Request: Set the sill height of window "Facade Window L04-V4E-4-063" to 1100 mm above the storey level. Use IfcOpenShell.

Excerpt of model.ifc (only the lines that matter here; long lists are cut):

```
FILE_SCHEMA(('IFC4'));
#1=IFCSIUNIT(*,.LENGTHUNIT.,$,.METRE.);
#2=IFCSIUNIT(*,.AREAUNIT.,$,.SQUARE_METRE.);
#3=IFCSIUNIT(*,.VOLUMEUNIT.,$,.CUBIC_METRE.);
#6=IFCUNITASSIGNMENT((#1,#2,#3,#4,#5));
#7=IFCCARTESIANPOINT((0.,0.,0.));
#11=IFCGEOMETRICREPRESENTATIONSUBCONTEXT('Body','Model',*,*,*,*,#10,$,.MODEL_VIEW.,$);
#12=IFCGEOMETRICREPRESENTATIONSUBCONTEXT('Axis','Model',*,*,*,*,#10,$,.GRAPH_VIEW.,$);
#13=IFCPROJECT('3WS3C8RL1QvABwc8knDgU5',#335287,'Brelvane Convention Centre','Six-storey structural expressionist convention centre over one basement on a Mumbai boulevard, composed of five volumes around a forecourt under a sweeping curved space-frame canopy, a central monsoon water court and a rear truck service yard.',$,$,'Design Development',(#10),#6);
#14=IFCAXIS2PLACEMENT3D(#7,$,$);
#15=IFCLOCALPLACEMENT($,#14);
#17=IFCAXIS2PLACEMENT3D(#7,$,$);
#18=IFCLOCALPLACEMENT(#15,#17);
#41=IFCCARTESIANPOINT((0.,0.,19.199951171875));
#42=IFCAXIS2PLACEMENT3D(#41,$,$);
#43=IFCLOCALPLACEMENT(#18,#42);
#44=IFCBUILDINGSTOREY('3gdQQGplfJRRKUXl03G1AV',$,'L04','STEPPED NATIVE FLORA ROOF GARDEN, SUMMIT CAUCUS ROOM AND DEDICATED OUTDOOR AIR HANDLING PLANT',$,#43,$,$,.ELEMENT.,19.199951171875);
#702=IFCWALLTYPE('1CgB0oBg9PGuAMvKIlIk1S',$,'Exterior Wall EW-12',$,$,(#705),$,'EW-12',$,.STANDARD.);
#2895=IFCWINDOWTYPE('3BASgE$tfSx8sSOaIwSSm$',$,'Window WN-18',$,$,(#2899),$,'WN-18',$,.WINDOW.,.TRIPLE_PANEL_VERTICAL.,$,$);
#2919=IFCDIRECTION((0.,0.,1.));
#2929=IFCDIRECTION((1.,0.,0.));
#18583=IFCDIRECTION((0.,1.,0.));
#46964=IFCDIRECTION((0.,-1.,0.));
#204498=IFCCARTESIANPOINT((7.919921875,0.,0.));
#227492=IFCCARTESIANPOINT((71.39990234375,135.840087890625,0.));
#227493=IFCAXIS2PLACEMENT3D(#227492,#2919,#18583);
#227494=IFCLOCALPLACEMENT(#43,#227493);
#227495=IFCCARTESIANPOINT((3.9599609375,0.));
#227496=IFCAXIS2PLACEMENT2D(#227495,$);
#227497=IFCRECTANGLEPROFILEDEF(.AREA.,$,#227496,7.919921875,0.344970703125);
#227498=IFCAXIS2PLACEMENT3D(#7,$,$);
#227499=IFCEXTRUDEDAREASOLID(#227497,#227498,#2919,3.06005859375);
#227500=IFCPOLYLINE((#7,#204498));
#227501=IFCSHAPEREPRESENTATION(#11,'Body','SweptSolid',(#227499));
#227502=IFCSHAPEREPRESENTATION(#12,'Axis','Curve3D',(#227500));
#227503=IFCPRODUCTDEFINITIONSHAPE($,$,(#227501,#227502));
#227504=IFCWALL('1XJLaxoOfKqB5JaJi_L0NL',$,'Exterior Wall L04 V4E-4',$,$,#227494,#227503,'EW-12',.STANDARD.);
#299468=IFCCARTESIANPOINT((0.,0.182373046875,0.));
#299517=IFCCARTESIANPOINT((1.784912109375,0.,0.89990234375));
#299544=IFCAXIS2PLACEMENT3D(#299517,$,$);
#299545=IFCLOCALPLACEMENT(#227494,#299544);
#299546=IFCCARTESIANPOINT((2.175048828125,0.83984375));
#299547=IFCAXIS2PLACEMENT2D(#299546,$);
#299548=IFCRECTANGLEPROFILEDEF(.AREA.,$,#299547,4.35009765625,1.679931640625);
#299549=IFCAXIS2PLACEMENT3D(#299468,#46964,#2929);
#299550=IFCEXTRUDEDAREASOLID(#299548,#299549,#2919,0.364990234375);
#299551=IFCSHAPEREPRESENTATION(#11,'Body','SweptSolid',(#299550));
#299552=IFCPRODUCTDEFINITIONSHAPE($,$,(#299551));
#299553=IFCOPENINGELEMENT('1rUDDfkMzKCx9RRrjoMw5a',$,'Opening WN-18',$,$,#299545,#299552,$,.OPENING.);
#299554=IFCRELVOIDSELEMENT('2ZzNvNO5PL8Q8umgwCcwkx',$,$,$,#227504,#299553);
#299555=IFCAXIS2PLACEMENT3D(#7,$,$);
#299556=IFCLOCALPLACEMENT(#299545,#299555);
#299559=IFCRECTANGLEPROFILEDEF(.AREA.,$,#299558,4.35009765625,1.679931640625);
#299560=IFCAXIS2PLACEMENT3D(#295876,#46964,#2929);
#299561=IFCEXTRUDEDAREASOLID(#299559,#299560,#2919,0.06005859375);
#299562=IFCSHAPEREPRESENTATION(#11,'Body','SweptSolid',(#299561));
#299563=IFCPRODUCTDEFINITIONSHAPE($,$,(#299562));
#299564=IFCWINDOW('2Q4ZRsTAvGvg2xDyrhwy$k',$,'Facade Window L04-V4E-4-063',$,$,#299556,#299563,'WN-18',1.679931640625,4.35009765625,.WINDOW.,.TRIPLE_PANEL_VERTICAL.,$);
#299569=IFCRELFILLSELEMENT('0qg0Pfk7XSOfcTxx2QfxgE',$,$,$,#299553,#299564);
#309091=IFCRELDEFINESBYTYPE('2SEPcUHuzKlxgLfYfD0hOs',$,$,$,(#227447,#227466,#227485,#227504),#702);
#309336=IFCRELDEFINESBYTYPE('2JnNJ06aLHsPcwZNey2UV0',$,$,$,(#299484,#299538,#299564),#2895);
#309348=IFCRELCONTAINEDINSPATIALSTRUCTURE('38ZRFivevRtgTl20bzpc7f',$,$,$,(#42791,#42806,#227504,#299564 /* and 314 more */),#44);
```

```python
import numpy as np
import ifcopenshell
import ifcopenshell.api.geometry
import ifcopenshell.geom
import ifcopenshell.util.element
import ifcopenshell.util.placement
import ifcopenshell.util.shape
import ifcopenshell.util.unit

model = ifcopenshell.open("model.ifc")
unit_scale = ifcopenshell.util.unit.calculate_unit_scale(model)

window = model.by_guid("2Q4ZRsTAvGvg2xDyrhwy$k")
opening = window.FillsVoids[0].RelatingOpeningElement
storey = ifcopenshell.util.element.get_container(window, ifc_class="IfcBuildingStorey")
level = ifcopenshell.util.placement.get_local_placement(storey.ObjectPlacement)[2, 3]

# The opening's origin need not be at the sill, so measure its lowest point.
shape = ifcopenshell.geom.create_shape(ifcopenshell.geom.settings(), opening)
bottom = ifcopenshell.util.shape.get_shape_bottom_elevation(shape, shape.geometry) / unit_scale
dz = level + 1.1 - bottom

shift = np.array([0.0, 0.0, dz])
# The window is placed relative to its opening, so it follows when the opening moves.
matrix = ifcopenshell.util.placement.get_local_placement(opening.ObjectPlacement)
matrix[:3, 3] += shift
ifcopenshell.api.geometry.edit_object_placement(
    model, product=opening, matrix=matrix, is_si=False, should_transform_children=True
)

print(f"moved by {dz * unit_scale:+.3f} m")

model.write("model-out.ifc")
```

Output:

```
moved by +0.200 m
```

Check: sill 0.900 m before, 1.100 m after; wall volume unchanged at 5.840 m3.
